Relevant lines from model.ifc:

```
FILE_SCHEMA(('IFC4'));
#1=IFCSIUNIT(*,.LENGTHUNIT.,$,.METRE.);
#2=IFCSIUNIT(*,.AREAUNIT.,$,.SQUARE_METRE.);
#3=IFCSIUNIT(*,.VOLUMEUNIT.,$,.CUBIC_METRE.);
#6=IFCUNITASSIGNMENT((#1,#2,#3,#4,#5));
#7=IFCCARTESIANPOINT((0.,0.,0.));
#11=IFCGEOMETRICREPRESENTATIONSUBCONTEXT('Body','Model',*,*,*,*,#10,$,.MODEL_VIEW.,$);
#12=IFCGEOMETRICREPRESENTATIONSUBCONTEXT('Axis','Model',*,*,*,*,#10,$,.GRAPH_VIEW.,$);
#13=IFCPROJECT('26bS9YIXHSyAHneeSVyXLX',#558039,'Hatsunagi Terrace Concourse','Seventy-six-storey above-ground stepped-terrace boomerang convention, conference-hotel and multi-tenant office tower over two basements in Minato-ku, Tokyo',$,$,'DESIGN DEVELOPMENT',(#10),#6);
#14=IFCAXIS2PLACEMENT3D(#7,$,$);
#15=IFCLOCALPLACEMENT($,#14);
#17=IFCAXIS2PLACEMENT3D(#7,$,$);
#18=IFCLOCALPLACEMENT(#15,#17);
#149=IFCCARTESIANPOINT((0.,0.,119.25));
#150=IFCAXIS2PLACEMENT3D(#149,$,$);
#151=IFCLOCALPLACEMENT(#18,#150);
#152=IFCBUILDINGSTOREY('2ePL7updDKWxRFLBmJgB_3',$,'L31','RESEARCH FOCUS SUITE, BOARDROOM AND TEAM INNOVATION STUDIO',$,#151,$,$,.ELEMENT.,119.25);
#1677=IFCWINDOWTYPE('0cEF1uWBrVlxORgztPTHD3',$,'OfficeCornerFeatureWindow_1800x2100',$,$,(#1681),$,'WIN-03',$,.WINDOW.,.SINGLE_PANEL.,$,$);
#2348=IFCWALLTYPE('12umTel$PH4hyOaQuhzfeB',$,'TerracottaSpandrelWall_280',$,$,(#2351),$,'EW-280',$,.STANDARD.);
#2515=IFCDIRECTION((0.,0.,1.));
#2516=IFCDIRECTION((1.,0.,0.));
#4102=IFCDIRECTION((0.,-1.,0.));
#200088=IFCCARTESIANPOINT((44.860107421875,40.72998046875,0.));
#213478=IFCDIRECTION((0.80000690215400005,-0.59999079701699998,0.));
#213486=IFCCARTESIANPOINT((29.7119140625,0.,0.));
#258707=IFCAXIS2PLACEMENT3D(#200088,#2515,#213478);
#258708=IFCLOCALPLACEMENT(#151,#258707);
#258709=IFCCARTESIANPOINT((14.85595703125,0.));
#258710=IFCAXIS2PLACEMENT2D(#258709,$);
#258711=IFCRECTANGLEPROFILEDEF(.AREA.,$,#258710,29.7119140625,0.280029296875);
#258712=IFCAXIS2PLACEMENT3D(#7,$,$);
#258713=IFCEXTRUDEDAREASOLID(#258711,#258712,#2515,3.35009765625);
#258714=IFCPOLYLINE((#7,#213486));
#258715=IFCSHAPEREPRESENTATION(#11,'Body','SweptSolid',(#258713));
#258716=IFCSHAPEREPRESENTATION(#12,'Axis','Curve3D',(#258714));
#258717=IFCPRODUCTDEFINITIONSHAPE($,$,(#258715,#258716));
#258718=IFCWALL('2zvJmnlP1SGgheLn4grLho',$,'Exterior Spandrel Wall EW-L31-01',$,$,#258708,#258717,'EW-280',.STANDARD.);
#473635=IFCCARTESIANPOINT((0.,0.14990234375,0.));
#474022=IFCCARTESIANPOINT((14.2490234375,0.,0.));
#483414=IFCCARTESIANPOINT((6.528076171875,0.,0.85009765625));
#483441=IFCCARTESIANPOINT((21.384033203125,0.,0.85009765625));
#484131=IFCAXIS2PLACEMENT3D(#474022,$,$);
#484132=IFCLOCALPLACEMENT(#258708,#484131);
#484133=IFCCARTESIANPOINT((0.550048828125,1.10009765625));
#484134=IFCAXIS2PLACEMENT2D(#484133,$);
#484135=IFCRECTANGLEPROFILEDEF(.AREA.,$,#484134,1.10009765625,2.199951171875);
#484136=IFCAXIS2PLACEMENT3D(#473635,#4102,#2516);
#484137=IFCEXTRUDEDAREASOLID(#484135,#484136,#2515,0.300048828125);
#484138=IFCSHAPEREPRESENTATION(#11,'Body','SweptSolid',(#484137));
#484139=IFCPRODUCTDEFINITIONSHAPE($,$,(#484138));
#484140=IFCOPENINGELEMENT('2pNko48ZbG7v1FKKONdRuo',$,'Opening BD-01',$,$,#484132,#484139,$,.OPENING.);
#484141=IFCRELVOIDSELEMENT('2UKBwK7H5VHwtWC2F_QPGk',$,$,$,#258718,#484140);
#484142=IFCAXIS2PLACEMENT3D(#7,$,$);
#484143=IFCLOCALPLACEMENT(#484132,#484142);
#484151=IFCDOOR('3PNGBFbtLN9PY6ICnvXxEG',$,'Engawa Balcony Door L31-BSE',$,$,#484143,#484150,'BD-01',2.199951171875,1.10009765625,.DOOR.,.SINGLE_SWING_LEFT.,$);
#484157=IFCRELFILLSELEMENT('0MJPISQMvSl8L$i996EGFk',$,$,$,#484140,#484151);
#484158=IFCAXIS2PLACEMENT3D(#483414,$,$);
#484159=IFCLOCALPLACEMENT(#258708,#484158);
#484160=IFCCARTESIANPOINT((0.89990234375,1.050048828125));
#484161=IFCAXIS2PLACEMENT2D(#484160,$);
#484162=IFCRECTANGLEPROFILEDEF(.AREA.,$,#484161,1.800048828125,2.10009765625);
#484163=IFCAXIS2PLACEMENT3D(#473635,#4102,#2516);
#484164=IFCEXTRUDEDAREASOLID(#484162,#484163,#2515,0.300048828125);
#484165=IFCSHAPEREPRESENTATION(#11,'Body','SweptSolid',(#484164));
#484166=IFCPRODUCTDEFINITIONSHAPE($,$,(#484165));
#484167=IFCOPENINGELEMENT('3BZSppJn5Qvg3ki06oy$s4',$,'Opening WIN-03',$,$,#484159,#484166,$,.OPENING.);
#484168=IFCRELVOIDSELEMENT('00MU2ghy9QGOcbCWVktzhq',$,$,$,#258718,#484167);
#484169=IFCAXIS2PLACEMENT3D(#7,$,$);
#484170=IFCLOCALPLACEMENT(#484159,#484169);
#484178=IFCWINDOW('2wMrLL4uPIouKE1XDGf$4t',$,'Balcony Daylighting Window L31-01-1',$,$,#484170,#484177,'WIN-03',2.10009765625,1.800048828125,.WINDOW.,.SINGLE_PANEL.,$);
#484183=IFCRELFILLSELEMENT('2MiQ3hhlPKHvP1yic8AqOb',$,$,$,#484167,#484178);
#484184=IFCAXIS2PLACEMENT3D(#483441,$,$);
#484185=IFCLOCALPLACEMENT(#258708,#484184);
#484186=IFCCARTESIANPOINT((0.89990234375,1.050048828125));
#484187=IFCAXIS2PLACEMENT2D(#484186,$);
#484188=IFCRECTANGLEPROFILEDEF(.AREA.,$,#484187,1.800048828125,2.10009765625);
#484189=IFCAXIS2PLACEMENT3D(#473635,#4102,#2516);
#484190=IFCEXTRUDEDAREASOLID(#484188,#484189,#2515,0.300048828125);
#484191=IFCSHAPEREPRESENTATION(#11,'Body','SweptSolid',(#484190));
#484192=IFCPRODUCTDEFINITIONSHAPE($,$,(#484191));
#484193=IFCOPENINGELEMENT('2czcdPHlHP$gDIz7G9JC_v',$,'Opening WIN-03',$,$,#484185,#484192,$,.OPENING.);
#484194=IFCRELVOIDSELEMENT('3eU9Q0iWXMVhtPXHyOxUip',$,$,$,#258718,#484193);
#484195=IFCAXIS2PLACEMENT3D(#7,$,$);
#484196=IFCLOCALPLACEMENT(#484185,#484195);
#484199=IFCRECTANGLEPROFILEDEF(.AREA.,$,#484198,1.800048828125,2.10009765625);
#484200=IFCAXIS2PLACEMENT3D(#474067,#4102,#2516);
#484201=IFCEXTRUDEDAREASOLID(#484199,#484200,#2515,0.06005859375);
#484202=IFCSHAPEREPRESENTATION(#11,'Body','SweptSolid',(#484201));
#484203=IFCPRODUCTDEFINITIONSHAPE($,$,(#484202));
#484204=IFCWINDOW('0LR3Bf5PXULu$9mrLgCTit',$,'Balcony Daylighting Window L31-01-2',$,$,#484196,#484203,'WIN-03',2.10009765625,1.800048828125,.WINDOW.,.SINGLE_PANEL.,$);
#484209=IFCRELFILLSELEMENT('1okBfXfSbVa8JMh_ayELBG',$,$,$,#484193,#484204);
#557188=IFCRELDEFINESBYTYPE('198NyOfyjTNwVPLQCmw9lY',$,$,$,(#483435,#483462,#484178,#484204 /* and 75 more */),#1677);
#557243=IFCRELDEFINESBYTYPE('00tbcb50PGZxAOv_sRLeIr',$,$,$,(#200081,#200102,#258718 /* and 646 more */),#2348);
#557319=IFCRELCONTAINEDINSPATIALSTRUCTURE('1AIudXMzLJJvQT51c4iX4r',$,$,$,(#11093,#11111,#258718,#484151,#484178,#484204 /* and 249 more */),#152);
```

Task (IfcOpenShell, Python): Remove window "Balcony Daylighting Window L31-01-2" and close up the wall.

```python
import ifcopenshell
import ifcopenshell.api.feature
import ifcopenshell.api.root
import ifcopenshell.geom
import ifcopenshell.util.shape

model = ifcopenshell.open("model.ifc")
settings = ifcopenshell.geom.settings()


def volume(element):
    """Net volume in cubic metres, openings subtracted."""
    shape = ifcopenshell.geom.create_shape(settings, element)
    return ifcopenshell.util.shape.get_volume(shape.geometry)


window = model.by_guid("0LR3Bf5PXULu$9mrLgCTit")
opening = window.FillsVoids[0].RelatingOpeningElement
wall = opening.VoidsElements[0].RelatingBuildingElement
before = volume(wall)

ifcopenshell.api.root.remove_product(model, product=window)
ifcopenshell.api.feature.remove_feature(model, feature=opening)

after = volume(wall)

print(f"wall volume {before:.3f} -> {after:.3f} m3")

model.write("model_edited.ifc")
```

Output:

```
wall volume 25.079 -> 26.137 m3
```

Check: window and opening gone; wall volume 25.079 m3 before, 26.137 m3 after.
